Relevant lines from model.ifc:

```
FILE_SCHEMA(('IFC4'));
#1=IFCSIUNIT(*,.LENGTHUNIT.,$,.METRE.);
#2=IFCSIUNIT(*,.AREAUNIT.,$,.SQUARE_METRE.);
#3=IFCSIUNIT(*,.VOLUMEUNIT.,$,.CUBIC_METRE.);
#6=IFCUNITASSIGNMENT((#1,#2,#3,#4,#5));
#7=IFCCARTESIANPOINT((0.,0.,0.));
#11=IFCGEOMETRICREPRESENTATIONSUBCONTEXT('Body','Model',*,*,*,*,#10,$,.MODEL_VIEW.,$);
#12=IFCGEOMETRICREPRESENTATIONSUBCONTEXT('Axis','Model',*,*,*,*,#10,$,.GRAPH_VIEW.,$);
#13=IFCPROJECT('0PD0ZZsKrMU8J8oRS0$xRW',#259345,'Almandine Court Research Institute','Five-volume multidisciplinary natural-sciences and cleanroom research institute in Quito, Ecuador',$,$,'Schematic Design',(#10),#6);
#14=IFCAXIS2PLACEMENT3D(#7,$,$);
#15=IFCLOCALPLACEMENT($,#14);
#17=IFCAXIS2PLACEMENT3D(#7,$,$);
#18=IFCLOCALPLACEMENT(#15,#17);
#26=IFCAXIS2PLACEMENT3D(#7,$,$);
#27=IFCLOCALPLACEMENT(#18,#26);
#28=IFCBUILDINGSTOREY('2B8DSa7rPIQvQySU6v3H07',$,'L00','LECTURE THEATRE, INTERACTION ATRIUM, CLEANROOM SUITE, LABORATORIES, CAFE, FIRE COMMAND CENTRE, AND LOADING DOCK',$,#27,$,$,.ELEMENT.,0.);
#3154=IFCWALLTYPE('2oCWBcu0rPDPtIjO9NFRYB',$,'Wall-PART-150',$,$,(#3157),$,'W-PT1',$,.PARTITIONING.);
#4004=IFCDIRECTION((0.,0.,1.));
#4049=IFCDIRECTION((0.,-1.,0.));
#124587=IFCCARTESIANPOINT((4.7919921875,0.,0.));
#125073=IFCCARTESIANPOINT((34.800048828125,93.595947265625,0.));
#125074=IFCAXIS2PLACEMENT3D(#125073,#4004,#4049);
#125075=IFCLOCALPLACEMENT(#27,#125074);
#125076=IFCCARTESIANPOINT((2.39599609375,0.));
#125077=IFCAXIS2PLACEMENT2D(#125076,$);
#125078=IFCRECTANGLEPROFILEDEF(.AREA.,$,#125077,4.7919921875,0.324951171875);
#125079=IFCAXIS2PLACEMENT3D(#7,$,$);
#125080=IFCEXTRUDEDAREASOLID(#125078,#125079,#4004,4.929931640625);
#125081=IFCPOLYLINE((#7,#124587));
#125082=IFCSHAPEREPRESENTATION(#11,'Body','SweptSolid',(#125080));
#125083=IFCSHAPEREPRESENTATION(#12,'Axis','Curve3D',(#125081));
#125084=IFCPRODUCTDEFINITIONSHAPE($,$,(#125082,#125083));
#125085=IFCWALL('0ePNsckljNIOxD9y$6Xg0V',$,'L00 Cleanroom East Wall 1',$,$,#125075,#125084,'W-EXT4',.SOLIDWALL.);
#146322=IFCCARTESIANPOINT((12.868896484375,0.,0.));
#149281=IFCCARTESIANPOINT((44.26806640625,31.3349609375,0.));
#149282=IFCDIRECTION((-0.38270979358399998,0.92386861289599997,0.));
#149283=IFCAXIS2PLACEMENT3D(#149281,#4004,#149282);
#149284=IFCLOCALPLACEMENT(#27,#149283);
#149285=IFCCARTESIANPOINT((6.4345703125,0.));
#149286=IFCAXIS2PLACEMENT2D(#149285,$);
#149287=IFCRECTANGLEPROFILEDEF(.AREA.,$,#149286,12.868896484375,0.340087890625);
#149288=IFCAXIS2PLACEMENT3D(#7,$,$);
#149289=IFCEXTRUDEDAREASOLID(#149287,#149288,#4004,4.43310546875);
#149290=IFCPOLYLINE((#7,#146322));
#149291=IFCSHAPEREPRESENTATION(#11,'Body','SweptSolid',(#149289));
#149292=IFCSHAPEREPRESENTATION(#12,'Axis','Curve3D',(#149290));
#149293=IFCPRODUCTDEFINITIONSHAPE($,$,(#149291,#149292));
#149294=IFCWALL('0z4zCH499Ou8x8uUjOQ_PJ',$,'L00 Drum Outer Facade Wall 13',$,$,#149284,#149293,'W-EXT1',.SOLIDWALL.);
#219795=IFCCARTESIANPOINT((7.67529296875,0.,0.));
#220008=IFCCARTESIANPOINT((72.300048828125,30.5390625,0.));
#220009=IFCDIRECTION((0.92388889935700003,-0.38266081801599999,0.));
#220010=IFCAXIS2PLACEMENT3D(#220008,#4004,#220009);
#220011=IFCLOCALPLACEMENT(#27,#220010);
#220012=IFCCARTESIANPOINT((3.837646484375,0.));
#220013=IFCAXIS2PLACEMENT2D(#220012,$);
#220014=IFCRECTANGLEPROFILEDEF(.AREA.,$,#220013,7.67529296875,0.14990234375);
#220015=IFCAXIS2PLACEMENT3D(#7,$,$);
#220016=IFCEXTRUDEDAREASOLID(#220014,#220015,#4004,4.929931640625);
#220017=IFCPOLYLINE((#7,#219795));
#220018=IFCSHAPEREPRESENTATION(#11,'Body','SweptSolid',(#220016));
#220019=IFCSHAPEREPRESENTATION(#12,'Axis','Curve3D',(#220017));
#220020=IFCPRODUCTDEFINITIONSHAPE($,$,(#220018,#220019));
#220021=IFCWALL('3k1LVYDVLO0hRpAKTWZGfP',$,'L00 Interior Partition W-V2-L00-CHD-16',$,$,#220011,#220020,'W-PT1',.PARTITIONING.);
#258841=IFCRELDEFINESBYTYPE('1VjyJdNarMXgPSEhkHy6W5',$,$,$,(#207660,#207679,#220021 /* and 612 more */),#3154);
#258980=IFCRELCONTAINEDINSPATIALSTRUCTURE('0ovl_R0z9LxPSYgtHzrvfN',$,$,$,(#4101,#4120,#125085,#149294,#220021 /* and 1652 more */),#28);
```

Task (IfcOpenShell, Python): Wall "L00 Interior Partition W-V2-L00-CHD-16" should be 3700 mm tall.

```python
import ifcopenshell
import ifcopenshell.geom
import ifcopenshell.util.representation
import ifcopenshell.util.shape
import ifcopenshell.util.unit

model = ifcopenshell.open("model.ifc")
unit_scale = ifcopenshell.util.unit.calculate_unit_scale(model)
settings = ifcopenshell.geom.settings()


def volume(element):
    """Net volume in cubic metres, openings subtracted."""
    shape = ifcopenshell.geom.create_shape(settings, element)
    return ifcopenshell.util.shape.get_volume(shape.geometry)


wall = model.by_guid("3k1LVYDVLO0hRpAKTWZGfP")
before = volume(wall)

body = ifcopenshell.util.representation.get_representation(wall, "Model", "Body")
solid = body.Items[0]
old_height = solid.Depth
solid.Depth = 3.7 / unit_scale
after = volume(wall)

print(f"height {old_height:g} -> {solid.Depth:g}, volume {before:.3f} -> {after:.3f} m3")

model.write("model_rev.ifc")
```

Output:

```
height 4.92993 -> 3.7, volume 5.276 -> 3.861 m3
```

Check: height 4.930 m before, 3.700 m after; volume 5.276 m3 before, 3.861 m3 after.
